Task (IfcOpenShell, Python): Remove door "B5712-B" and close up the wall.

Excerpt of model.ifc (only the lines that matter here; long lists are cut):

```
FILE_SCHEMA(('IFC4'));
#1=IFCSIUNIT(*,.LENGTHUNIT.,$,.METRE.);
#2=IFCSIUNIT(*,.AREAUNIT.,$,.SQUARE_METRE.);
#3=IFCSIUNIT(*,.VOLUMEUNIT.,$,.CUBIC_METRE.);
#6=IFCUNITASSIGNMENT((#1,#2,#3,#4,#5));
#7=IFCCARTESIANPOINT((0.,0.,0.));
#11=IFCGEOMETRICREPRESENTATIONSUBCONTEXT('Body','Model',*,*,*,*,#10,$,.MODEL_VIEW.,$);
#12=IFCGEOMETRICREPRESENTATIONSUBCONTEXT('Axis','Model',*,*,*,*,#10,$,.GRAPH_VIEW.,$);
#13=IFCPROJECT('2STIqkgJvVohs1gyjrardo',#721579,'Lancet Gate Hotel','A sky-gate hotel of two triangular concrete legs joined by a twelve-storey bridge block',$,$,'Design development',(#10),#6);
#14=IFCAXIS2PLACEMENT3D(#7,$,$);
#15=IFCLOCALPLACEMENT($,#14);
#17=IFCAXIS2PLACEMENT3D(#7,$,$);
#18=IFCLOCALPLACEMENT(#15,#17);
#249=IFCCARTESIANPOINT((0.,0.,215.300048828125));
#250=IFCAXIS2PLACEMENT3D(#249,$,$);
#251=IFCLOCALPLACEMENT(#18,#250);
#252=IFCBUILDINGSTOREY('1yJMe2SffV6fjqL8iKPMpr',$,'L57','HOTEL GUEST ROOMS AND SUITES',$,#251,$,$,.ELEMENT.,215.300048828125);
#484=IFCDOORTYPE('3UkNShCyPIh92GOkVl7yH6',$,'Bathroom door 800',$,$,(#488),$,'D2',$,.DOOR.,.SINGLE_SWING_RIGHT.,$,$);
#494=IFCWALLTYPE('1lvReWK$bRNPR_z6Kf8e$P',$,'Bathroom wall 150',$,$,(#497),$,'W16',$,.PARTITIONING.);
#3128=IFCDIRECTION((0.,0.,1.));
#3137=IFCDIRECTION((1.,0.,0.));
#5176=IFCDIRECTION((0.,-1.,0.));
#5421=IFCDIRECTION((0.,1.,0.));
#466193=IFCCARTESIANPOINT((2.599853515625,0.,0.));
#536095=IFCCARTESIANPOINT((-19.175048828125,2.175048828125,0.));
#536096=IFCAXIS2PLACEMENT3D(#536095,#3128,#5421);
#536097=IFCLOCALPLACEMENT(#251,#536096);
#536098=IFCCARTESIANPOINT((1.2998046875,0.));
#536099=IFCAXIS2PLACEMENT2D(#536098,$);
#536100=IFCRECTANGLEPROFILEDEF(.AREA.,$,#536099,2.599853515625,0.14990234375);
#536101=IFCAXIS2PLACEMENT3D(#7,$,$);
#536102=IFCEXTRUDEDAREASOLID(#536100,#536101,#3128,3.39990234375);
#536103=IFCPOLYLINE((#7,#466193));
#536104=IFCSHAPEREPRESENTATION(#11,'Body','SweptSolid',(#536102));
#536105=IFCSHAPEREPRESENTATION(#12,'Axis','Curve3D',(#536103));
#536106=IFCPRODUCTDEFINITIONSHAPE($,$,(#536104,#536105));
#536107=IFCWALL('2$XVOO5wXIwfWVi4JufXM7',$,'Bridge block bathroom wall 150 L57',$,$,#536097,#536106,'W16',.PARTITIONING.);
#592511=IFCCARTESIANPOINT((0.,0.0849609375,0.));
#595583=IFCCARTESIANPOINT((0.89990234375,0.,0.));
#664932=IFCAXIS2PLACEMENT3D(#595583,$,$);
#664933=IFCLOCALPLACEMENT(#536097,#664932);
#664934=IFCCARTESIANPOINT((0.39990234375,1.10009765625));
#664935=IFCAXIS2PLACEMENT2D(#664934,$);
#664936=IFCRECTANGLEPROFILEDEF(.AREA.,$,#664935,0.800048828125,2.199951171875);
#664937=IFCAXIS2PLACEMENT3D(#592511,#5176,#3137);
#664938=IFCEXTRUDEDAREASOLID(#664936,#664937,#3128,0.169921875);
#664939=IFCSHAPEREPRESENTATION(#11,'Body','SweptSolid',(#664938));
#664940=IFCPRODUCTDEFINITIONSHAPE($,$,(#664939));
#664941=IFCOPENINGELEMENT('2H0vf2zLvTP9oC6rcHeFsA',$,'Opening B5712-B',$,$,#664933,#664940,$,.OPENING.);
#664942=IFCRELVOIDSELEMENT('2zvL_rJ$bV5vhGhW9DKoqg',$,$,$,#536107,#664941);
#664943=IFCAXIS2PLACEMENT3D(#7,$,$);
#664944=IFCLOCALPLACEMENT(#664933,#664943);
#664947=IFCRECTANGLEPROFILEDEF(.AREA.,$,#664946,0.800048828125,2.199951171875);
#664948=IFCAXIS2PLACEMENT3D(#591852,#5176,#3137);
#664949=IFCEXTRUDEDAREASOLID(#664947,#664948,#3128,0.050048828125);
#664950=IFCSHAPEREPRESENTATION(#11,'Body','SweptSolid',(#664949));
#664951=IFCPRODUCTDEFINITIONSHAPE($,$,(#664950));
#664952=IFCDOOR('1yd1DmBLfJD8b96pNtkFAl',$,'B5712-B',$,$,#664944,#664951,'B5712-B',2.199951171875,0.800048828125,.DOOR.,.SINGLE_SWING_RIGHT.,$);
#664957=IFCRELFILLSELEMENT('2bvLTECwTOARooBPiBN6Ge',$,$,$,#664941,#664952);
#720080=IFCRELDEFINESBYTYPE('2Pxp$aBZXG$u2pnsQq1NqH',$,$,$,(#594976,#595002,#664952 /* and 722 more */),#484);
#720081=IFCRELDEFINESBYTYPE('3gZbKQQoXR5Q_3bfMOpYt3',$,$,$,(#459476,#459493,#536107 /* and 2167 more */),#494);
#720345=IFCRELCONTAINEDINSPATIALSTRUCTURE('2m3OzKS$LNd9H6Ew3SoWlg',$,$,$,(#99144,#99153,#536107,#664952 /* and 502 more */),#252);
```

```python
import ifcopenshell
import ifcopenshell.api.feature
import ifcopenshell.api.root
import ifcopenshell.geom
import ifcopenshell.util.shape

model = ifcopenshell.open("model.ifc")
settings = ifcopenshell.geom.settings()


def volume(element):
    """Net volume in cubic metres, openings subtracted."""
    shape = ifcopenshell.geom.create_shape(settings, element)
    return ifcopenshell.util.shape.get_volume(shape.geometry)


door = model.by_id(664952)
opening = door.FillsVoids[0].RelatingOpeningElement
wall = opening.VoidsElements[0].RelatingBuildingElement
before = volume(wall)

ifcopenshell.api.root.remove_product(model, product=door)
ifcopenshell.api.feature.remove_feature(model, feature=opening)

after = volume(wall)

print(f"wall volume {before:.3f} -> {after:.3f} m3")

model.write("model_updated.ifc")
```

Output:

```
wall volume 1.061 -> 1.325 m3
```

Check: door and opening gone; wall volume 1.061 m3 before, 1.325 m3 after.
